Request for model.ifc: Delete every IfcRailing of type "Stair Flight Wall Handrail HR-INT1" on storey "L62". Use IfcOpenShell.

First a look at what the model holds.

```python
import ifcopenshell
import ifcopenshell.util.element

model = ifcopenshell.open("model.ifc")
print(model.schema)
storey = next(s for s in model.by_type("IfcBuildingStorey") if s.Name == "L62")
railings = [e for e in ifcopenshell.util.element.get_decomposition(storey) if e.is_a("IfcRailing")]
seen = {}
for e in railings:
    element_type = ifcopenshell.util.element.get_type(e)
    name = element_type.Name if element_type not in (None, e) else None
    seen[name] = seen.get(name, 0) + 1
for name, count in sorted(seen.items(), key=str):
    print(count, "x", name)
```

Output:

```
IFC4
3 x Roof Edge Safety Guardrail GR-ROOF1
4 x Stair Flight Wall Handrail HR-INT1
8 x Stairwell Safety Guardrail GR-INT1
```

```python
import ifcopenshell
import ifcopenshell.api.root
import ifcopenshell.util.element

model = ifcopenshell.open("model.ifc")

storey = next(s for s in model.by_type("IfcBuildingStorey") if s.Name == "L62")
railings = [e for e in ifcopenshell.util.element.get_decomposition(storey) if e.is_a("IfcRailing")]
targets = [e for e in railings if (t := ifcopenshell.util.element.get_type(e)) not in (None, e) and t.Name == "Stair Flight Wall Handrail HR-INT1"]

for e in targets:
    ifcopenshell.api.root.remove_product(model, product=e)
print(len(targets), "removed")

model.write("model_v2.ifc")
```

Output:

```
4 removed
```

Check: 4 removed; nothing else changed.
